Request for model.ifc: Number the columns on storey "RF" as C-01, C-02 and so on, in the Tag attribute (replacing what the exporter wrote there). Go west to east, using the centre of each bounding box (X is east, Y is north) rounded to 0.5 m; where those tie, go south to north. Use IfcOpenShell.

First a look at what the model holds.

```python
import ifcopenshell
import ifcopenshell.util.element
import ifcopenshell.util.placement

model = ifcopenshell.open("model.ifc")
print(model.schema)
storey = next(s for s in model.by_type("IfcBuildingStorey") if s.Name == "RF")
columns = [e for e in ifcopenshell.util.element.get_decomposition(storey) if e.is_a("IfcColumn")]
for e in sorted(columns, key=lambda e: e.id()):
    origin = ifcopenshell.util.placement.get_local_placement(e.ObjectPlacement)[:3, 3]
    print(e.id(), e.Tag, e.Name, origin.round(2) + 0.0, sep=" | ")
```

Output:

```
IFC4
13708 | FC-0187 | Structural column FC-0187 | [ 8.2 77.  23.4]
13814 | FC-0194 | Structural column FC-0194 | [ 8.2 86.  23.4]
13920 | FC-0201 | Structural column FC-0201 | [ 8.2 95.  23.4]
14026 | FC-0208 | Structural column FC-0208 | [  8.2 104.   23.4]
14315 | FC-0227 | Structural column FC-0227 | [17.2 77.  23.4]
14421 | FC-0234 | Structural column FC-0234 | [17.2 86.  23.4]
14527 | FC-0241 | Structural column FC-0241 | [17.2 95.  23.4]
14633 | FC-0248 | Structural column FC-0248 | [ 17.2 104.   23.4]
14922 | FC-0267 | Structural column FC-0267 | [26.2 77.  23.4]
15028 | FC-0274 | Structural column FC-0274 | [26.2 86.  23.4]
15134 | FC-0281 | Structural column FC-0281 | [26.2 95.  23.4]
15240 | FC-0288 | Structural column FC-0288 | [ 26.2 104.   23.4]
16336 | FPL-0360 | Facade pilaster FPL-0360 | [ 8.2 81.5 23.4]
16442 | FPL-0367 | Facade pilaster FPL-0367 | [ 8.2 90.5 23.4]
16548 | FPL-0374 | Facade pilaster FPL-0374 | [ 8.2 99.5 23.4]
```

```python
import ifcopenshell
import ifcopenshell.geom
import ifcopenshell.util.element
import ifcopenshell.util.shape

model = ifcopenshell.open("model.ifc")
settings = ifcopenshell.geom.settings()
settings.set("use-world-coords", True)


def centre(element):
    shape = ifcopenshell.geom.create_shape(settings, element)
    return ifcopenshell.util.shape.get_bbox_centroid(shape.geometry)


storey = next(s for s in model.by_type("IfcBuildingStorey") if s.Name == "RF")
columns = [e for e in ifcopenshell.util.element.get_decomposition(storey) if e.is_a("IfcColumn")]

# Insertion points can sit at a corner or the storey origin, so sort by the geometry (in metres).
centres = {e: centre(e) for e in columns}
columns.sort(key=lambda e: (round(centres[e][0] / 0.5), centres[e][1]))

for i, e in enumerate(columns, start=1):
    number = f"C-{i:02d}"
    e.Tag = number
    print(e.id(), number)

model.write("model-out.ifc")
```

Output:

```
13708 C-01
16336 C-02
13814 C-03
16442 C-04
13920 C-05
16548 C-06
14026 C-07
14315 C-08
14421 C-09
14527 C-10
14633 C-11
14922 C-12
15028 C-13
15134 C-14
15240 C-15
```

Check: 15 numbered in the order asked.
